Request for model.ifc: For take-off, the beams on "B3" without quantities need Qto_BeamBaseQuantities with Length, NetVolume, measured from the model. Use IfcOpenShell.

First a look at what the model holds.

```python
import ifcopenshell
import ifcopenshell.util.element
import ifcopenshell.util.unit

model = ifcopenshell.open("model.ifc")
print(model.schema)
for unit_type in ("LENGTHUNIT", "AREAUNIT", "VOLUMEUNIT"):
    print(unit_type, ifcopenshell.util.unit.calculate_unit_scale(model, unit_type))
storey = next(s for s in model.by_type("IfcBuildingStorey") if s.Name == "B3")
beams = [e for e in ifcopenshell.util.element.get_decomposition(storey) if e.is_a("IfcBeam")]
for e in sorted(beams, key=lambda e: e.id()):
    print(e.id(), e.is_a(), e.Name, list(ifcopenshell.util.element.get_psets(e, qtos_only=True)), sep=" | ")
```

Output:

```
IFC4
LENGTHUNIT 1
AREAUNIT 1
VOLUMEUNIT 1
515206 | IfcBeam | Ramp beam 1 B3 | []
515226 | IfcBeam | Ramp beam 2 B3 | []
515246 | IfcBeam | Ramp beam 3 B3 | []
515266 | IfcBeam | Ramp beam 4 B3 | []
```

```python
import ifcopenshell
import ifcopenshell.api.pset
import ifcopenshell.geom
import ifcopenshell.util.element
import ifcopenshell.util.shape
import ifcopenshell.util.unit

model = ifcopenshell.open("model.ifc")
unit_scale = ifcopenshell.util.unit.calculate_unit_scale(model)
volume_scale = ifcopenshell.util.unit.calculate_unit_scale(model, "VOLUMEUNIT")
settings = ifcopenshell.geom.settings()

storey = next(s for s in model.by_type("IfcBuildingStorey") if s.Name == "B3")
beams = [e for e in ifcopenshell.util.element.get_decomposition(storey) if e.is_a("IfcBeam")]

for e in sorted(beams, key=lambda e: e.id()):
    if ifcopenshell.util.element.get_psets(e, qtos_only=True, should_inherit=False):
        continue
    # Geometry comes back in metres, in the element's own axes.
    shape = ifcopenshell.geom.create_shape(settings, e)
    values = {
        "Length": ifcopenshell.util.shape.get_max_xyz(shape.geometry) / unit_scale,
        "NetVolume": ifcopenshell.util.shape.get_volume(shape.geometry) / volume_scale,
    }
    qto = ifcopenshell.api.pset.add_qto(model, product=e, name="Qto_BeamBaseQuantities")
    ifcopenshell.api.pset.edit_qto(model, qto=qto, properties=values)
    print(e.id(), {k: round(v, 3) for k, v in values.items()})

model.write("model_edited.ifc")
```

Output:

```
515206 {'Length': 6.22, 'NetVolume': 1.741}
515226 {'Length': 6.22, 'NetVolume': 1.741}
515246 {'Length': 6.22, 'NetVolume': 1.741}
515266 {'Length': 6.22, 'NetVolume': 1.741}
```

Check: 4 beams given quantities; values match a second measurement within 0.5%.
